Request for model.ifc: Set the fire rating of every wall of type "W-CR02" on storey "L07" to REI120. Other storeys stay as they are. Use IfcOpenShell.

First a look at what the model holds.

```python
import ifcopenshell
import ifcopenshell.util.element

model = ifcopenshell.open("model.ifc")
print(model.schema)
storey = next(s for s in model.by_type("IfcBuildingStorey") if s.Name == "L07")
walls = [e for e in ifcopenshell.util.element.get_decomposition(storey) if e.is_a("IfcWall")]
seen = {}
for e in walls:
    element_type = ifcopenshell.util.element.get_type(e)
    key = (element_type.Name if element_type != e and element_type else None, ifcopenshell.util.element.get_pset(e, "Pset_WallCommon", "FireRating"))
    seen[key] = seen.get(key, 0) + 1
for (name, value), count in sorted(seen.items(), key=str):
    print(count, "x", name, "|", value)
```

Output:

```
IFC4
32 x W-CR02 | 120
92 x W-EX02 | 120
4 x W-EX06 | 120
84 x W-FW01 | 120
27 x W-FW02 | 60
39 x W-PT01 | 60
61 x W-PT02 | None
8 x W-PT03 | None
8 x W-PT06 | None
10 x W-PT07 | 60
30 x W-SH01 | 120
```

```python
import ifcopenshell
import ifcopenshell.api.pset
import ifcopenshell.util.element

model = ifcopenshell.open("model.ifc")

storey = next(s for s in model.by_type("IfcBuildingStorey") if s.Name == "L07")
walls = [e for e in ifcopenshell.util.element.get_decomposition(storey) if e.is_a("IfcWall")]

count = 0
for e in walls:
    element_type = ifcopenshell.util.element.get_type(e)
    if element_type in (None, e) or element_type.Name != "W-CR02":
        continue
    # add_pset returns the element's existing set when there is one.
    pset = ifcopenshell.api.pset.add_pset(model, product=e, name="Pset_WallCommon")
    ifcopenshell.api.pset.edit_pset(model, pset=pset, properties={"FireRating": "REI120"})
    count += 1

print(count, "walls updated")

model.write("model-out.ifc")
```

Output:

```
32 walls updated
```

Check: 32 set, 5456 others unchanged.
